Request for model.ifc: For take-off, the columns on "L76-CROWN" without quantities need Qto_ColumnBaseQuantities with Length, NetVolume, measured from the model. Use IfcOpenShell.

First a look at what the model holds.

```python
import ifcopenshell
import ifcopenshell.util.element
import ifcopenshell.util.unit

model = ifcopenshell.open("model.ifc")
print(model.schema)
for unit_type in ("LENGTHUNIT", "AREAUNIT", "VOLUMEUNIT"):
    print(unit_type, ifcopenshell.util.unit.calculate_unit_scale(model, unit_type))
storey = next(s for s in model.by_type("IfcBuildingStorey") if s.Name == "L76-CROWN")
columns = [e for e in ifcopenshell.util.element.get_decomposition(storey) if e.is_a("IfcColumn")]
for e in sorted(columns, key=lambda e: e.id()):
    print(e.id(), e.is_a(), e.Name, list(ifcopenshell.util.element.get_psets(e, qtos_only=True)), sep=" | ")
```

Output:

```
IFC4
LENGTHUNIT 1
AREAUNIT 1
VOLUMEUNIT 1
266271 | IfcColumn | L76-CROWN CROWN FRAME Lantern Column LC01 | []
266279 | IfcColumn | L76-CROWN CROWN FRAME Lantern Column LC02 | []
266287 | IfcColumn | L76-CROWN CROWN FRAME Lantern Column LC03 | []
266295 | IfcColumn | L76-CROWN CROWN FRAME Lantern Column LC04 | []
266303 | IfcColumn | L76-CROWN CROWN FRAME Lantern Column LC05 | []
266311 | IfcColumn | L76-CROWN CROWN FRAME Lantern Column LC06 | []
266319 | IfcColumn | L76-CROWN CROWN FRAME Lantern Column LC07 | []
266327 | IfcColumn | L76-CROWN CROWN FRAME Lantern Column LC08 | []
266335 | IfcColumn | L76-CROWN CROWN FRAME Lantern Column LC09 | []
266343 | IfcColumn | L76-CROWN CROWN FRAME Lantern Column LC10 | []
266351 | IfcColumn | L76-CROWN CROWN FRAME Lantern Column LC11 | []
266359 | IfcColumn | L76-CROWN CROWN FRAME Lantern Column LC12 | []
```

```python
import ifcopenshell
import ifcopenshell.api.pset
import ifcopenshell.geom
import ifcopenshell.util.element
import ifcopenshell.util.shape
import ifcopenshell.util.unit

model = ifcopenshell.open("model.ifc")
unit_scale = ifcopenshell.util.unit.calculate_unit_scale(model)
volume_scale = ifcopenshell.util.unit.calculate_unit_scale(model, "VOLUMEUNIT")
settings = ifcopenshell.geom.settings()

storey = next(s for s in model.by_type("IfcBuildingStorey") if s.Name == "L76-CROWN")
columns = [e for e in ifcopenshell.util.element.get_decomposition(storey) if e.is_a("IfcColumn")]

for e in sorted(columns, key=lambda e: e.id()):
    if ifcopenshell.util.element.get_psets(e, qtos_only=True, should_inherit=False):
        continue
    # Geometry comes back in metres, in the element's own axes.
    shape = ifcopenshell.geom.create_shape(settings, e)
    values = {
        "Length": ifcopenshell.util.shape.get_z(shape.geometry) / unit_scale,
        "NetVolume": ifcopenshell.util.shape.get_volume(shape.geometry) / volume_scale,
    }
    qto = ifcopenshell.api.pset.add_qto(model, product=e, name="Qto_ColumnBaseQuantities")
    ifcopenshell.api.pset.edit_qto(model, qto=qto, properties=values)
    print(e.id(), {k: round(v, 3) for k, v in values.items()})

model.write("model_v2.ifc")
```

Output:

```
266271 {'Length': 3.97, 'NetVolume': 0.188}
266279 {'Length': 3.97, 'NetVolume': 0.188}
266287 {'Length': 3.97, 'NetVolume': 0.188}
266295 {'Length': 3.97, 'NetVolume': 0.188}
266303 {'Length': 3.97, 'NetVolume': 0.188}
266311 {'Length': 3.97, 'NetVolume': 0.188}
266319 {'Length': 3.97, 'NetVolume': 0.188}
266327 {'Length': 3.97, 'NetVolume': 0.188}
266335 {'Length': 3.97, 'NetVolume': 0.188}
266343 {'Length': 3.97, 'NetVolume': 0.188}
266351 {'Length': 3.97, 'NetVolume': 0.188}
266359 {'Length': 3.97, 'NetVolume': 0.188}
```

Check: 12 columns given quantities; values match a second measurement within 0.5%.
